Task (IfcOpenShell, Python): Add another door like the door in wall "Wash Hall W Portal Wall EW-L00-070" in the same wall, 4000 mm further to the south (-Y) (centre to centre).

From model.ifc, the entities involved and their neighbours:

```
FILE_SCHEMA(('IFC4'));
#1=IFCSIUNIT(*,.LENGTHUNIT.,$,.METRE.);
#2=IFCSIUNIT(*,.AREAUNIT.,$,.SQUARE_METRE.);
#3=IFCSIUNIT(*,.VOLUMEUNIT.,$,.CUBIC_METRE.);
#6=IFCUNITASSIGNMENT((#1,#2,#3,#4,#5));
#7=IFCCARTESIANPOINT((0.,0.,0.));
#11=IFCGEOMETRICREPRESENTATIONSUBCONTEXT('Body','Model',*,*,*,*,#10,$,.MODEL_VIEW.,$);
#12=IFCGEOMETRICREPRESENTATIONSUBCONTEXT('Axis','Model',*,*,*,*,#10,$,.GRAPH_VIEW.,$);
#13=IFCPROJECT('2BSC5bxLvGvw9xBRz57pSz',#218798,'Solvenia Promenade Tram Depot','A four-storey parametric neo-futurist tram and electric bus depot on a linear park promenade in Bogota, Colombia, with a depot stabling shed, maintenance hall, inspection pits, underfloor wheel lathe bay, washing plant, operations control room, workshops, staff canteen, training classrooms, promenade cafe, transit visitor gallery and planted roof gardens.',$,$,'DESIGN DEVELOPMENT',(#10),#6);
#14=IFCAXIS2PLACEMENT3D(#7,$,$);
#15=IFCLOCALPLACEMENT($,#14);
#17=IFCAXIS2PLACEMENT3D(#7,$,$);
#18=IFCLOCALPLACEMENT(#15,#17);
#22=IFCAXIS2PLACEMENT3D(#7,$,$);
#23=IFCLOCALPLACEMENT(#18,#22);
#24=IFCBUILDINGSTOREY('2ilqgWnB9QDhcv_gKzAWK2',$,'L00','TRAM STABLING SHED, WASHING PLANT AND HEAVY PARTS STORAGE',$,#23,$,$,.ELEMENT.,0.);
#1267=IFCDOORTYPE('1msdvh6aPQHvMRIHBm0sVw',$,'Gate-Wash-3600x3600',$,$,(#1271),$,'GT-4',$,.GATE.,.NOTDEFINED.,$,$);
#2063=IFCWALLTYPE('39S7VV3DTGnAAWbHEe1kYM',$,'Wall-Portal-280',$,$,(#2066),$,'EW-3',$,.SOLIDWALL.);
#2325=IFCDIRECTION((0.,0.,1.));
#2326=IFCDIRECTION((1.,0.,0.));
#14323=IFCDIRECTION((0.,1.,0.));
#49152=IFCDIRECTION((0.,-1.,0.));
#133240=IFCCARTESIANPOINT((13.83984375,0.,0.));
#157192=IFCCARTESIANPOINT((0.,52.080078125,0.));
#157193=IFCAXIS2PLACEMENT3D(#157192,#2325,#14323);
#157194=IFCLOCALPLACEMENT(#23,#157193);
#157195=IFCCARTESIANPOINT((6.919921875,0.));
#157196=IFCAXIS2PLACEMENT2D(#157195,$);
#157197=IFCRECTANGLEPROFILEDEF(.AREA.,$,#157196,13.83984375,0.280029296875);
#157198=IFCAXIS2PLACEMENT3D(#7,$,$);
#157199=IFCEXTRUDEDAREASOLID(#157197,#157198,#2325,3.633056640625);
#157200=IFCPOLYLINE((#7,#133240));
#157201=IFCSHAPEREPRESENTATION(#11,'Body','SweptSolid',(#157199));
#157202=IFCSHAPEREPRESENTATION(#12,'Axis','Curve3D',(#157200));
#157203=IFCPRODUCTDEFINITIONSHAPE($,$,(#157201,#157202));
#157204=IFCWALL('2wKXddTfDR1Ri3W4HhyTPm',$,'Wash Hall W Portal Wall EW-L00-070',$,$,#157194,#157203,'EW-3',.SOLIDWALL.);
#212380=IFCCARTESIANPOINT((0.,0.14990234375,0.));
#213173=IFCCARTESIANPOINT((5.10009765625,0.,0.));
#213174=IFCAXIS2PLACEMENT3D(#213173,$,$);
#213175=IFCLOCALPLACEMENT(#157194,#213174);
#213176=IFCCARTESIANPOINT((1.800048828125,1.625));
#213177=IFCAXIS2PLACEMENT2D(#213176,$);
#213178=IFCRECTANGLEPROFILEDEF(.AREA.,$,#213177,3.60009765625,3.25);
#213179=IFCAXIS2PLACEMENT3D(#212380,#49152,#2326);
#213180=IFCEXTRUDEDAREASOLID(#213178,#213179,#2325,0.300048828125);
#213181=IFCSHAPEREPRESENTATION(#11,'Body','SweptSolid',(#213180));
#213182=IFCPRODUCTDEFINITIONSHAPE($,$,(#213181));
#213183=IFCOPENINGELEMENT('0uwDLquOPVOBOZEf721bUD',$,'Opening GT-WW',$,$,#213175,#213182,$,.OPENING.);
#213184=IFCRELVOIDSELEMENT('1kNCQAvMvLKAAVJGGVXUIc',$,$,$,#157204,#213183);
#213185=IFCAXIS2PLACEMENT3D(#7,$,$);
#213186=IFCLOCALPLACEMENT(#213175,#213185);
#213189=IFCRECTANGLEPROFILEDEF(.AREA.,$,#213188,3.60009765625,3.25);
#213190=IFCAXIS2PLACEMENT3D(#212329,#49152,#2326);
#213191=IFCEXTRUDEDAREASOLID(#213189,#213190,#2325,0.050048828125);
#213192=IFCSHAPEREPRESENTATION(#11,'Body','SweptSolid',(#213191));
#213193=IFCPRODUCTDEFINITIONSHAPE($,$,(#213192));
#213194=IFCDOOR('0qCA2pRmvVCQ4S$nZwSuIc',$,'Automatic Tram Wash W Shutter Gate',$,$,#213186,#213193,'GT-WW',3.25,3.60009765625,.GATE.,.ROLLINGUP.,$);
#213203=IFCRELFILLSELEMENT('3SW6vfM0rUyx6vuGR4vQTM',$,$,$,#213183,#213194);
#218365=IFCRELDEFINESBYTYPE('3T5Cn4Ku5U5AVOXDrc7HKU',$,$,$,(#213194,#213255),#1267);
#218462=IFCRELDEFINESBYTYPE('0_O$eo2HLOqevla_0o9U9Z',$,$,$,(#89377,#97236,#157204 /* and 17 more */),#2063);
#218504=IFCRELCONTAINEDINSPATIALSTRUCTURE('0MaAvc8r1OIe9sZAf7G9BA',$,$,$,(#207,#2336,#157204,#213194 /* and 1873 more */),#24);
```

```python
import ifcopenshell
import ifcopenshell.api.feature
import ifcopenshell.api.geometry
import ifcopenshell.api.root
import ifcopenshell.geom
import ifcopenshell.util.element
import ifcopenshell.util.placement
import ifcopenshell.util.shape

model = ifcopenshell.open("model.ifc")
settings = ifcopenshell.geom.settings()


def volume(element):
    """Net volume in cubic metres, openings subtracted."""
    shape = ifcopenshell.geom.create_shape(settings, element)
    return ifcopenshell.util.shape.get_volume(shape.geometry)


door = model.by_id(213194)
opening = door.FillsVoids[0].RelatingOpeningElement
wall = opening.VoidsElements[0].RelatingBuildingElement
before = volume(wall)
shift = ifcopenshell.util.placement.get_local_placement(wall.ObjectPlacement)[:3, 0] * -4.0

# copy_class copies the void relationship, type, container and properties, but no geometry.
new_opening = ifcopenshell.api.root.copy_class(model, product=opening)
new_opening.Representation = ifcopenshell.util.element.copy_deep(
    model, opening.Representation, exclude=["IfcGeometricRepresentationContext", "IfcRepresentationMap"]
)
new_door = ifcopenshell.api.root.copy_class(model, product=door)
new_door.Representation = ifcopenshell.util.element.copy_deep(
    model, door.Representation, exclude=["IfcGeometricRepresentationContext", "IfcRepresentationMap"]
)
new_door.Tag = None
ifcopenshell.api.feature.add_filling(model, opening=new_opening, element=new_door)

for old, new in ((opening, new_opening), (door, new_door)):
    matrix = ifcopenshell.util.placement.get_local_placement(old.ObjectPlacement)
    matrix[:3, 3] += shift
    ifcopenshell.api.geometry.edit_object_placement(model, product=new, matrix=matrix, is_si=False)

after = volume(wall)

print(f"wall volume {before:.3f} -> {after:.3f} m3")

model.write("model_v2.ifc")
```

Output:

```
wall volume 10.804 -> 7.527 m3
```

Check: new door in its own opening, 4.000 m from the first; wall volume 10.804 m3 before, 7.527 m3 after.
